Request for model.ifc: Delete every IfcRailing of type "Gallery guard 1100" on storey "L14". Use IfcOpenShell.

First a look at what the model holds.

```python
import ifcopenshell
import ifcopenshell.util.element

model = ifcopenshell.open("model.ifc")
print(model.schema)
storey = next(s for s in model.by_type("IfcBuildingStorey") if s.Name == "L14")
railings = [e for e in ifcopenshell.util.element.get_decomposition(storey) if e.is_a("IfcRailing")]
seen = {}
for e in railings:
    element_type = ifcopenshell.util.element.get_type(e)
    name = element_type.Name if element_type not in (None, e) else None
    seen[name] = seen.get(name, 0) + 1
for name, count in sorted(seen.items(), key=str):
    print(count, "x", name)
```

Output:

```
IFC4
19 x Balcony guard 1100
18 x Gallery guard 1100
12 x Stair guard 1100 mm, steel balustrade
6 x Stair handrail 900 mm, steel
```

```python
import ifcopenshell
import ifcopenshell.api.root
import ifcopenshell.util.element

model = ifcopenshell.open("model.ifc")

storey = next(s for s in model.by_type("IfcBuildingStorey") if s.Name == "L14")
railings = [e for e in ifcopenshell.util.element.get_decomposition(storey) if e.is_a("IfcRailing")]
targets = [e for e in railings if (t := ifcopenshell.util.element.get_type(e)) not in (None, e) and t.Name == "Gallery guard 1100"]

for e in targets:
    ifcopenshell.api.root.remove_product(model, product=e)
print(len(targets), "removed")

model.write("model_rev.ifc")
```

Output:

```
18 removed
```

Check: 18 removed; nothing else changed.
